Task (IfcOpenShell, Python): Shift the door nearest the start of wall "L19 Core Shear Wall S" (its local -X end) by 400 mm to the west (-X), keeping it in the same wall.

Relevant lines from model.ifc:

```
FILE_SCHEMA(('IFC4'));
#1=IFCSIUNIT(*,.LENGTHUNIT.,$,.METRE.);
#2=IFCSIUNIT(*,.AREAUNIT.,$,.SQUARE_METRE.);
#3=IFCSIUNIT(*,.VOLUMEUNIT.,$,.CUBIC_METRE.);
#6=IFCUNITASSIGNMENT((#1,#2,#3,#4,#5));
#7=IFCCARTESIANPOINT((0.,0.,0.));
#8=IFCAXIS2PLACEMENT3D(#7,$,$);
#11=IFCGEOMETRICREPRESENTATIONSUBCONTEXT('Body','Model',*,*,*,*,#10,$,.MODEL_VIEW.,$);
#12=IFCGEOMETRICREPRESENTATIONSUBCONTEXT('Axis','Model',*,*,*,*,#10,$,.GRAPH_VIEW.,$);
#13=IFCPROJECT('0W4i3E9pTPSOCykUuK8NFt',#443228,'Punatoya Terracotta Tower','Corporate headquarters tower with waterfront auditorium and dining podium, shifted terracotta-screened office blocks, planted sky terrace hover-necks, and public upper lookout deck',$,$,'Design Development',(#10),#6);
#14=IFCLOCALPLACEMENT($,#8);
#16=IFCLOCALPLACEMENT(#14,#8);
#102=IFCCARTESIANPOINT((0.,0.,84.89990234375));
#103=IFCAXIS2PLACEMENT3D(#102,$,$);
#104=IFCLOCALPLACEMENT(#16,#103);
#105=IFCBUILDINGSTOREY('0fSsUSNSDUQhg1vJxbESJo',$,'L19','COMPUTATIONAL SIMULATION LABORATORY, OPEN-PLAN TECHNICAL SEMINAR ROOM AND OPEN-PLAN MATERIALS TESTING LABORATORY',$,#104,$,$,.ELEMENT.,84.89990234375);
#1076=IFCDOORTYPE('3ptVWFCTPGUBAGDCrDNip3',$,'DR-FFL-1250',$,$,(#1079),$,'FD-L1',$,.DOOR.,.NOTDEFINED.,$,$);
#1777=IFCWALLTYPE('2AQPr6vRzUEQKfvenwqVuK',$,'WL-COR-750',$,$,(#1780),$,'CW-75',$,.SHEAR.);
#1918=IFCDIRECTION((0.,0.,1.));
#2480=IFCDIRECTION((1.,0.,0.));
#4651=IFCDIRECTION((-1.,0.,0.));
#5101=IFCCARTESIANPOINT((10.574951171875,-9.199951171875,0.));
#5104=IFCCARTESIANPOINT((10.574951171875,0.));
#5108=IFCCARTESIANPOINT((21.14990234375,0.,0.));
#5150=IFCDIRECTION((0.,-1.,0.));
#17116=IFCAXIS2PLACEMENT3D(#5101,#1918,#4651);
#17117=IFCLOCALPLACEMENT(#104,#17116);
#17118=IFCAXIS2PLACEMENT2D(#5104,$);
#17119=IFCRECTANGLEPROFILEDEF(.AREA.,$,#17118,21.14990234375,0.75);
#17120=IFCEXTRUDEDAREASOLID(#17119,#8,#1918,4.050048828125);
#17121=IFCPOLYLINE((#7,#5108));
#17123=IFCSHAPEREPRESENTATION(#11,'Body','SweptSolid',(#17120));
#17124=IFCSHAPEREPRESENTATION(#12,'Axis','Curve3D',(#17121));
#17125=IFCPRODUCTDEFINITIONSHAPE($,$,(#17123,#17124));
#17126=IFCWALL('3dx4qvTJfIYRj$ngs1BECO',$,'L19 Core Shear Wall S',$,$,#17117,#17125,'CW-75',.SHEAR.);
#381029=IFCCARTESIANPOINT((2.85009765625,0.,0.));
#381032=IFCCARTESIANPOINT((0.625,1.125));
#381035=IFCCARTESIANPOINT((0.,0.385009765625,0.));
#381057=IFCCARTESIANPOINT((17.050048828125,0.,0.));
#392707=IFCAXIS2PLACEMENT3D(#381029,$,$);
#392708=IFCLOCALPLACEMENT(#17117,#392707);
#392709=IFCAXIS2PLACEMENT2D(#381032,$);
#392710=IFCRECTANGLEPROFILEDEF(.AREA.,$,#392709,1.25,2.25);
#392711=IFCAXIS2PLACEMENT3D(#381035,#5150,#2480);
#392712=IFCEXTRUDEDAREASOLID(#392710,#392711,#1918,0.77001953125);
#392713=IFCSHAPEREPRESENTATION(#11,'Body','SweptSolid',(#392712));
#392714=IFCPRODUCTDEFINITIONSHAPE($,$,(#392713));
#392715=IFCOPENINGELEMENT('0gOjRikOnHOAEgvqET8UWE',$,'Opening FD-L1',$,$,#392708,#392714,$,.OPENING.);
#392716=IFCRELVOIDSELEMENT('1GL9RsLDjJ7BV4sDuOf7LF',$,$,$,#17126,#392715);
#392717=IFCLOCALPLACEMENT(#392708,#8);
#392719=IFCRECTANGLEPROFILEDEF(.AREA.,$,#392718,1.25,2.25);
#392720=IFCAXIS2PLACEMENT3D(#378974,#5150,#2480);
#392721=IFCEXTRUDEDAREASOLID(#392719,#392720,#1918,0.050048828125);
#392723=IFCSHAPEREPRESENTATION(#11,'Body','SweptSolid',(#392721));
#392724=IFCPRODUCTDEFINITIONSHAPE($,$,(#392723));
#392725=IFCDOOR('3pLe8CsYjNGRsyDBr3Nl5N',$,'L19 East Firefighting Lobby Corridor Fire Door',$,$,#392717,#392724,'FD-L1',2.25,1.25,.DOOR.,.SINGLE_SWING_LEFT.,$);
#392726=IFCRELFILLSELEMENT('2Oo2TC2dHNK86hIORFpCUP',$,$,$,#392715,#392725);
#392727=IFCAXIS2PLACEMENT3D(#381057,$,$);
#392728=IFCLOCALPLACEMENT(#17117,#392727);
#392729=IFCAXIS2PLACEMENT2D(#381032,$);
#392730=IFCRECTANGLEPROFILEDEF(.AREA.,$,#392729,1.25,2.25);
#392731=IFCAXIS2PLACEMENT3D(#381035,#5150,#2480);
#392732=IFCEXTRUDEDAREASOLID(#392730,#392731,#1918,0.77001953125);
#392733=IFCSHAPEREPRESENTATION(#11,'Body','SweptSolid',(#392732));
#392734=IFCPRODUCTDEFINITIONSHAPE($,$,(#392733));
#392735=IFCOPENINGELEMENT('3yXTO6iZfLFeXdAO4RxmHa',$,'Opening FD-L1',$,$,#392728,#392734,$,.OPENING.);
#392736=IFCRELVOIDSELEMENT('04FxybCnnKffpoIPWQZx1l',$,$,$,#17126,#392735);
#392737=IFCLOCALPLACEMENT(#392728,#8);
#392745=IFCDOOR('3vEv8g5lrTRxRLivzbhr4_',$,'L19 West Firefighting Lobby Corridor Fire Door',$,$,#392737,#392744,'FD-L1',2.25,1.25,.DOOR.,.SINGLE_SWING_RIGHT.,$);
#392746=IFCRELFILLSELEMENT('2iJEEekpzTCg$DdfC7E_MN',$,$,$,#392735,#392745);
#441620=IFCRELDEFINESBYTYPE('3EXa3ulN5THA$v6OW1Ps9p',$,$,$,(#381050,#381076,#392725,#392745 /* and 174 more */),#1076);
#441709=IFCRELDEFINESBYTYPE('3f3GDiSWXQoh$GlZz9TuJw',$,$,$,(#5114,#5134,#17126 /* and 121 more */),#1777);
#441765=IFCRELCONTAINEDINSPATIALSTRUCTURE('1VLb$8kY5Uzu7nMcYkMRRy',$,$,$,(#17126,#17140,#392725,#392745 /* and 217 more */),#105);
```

```python
import ifcopenshell
import ifcopenshell.api.geometry
import ifcopenshell.util.placement

model = ifcopenshell.open("model.ifc")

door = model.by_guid("3pLe8CsYjNGRsyDBr3Nl5N")
opening = door.FillsVoids[0].RelatingOpeningElement
wall = opening.VoidsElements[0].RelatingBuildingElement

wall_matrix = ifcopenshell.util.placement.get_local_placement(wall.ObjectPlacement)
shift = wall_matrix[:3, 0] * 0.4
before = ifcopenshell.util.placement.get_local_placement(door.ObjectPlacement)[:3, 3].copy()

# The door is placed relative to its opening, so it follows when the opening moves.
matrix = ifcopenshell.util.placement.get_local_placement(opening.ObjectPlacement)
matrix[:3, 3] += shift
ifcopenshell.api.geometry.edit_object_placement(
    model, product=opening, matrix=matrix, is_si=False, should_transform_children=True
)

after = ifcopenshell.util.placement.get_local_placement(door.ObjectPlacement)[:3, 3]
print("door moved by", (after - before).round(3) + 0.0)

model.write("model_v2.ifc")
```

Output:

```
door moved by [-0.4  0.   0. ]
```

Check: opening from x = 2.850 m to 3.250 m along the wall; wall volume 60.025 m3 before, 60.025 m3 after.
